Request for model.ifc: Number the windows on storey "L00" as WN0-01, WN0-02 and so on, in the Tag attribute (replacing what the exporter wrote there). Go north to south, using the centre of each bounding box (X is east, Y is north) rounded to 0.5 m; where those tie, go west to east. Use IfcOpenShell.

First a look at what the model holds.

```python
import ifcopenshell
import ifcopenshell.util.element
import ifcopenshell.util.placement

model = ifcopenshell.open("model.ifc")
print(model.schema)
storey = next(s for s in model.by_type("IfcBuildingStorey") if s.Name == "L00")
windows = [e for e in ifcopenshell.util.element.get_decomposition(storey) if e.is_a("IfcWindow")]
for e in sorted(windows, key=lambda e: e.id()):
    origin = ifcopenshell.util.placement.get_local_placement(e.ObjectPlacement)[:3, 3]
    print(e.id(), e.Tag, e.Name, origin.round(2) + 0.0, sep=" | ")
```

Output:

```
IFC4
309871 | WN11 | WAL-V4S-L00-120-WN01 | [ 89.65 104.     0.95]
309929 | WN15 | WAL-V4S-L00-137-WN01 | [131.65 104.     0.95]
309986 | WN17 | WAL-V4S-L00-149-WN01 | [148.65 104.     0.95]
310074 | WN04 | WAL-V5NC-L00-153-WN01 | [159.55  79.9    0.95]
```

```python
import ifcopenshell
import ifcopenshell.geom
import ifcopenshell.util.element
import ifcopenshell.util.shape

model = ifcopenshell.open("model.ifc")
settings = ifcopenshell.geom.settings()
settings.set("use-world-coords", True)


def centre(element):
    shape = ifcopenshell.geom.create_shape(settings, element)
    return ifcopenshell.util.shape.get_bbox_centroid(shape.geometry)


storey = next(s for s in model.by_type("IfcBuildingStorey") if s.Name == "L00")
windows = [e for e in ifcopenshell.util.element.get_decomposition(storey) if e.is_a("IfcWindow")]

# Insertion points can sit at a corner or the storey origin, so sort by the geometry (in metres).
centres = {e: centre(e) for e in windows}
windows.sort(key=lambda e: (-round(centres[e][1] / 0.5), centres[e][0]))

for i, e in enumerate(windows, start=1):
    number = f"WN0-{i:02d}"
    e.Tag = number
    print(e.id(), number)

model.write("model_updated.ifc")
```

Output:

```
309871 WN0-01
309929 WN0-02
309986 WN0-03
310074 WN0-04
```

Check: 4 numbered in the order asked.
